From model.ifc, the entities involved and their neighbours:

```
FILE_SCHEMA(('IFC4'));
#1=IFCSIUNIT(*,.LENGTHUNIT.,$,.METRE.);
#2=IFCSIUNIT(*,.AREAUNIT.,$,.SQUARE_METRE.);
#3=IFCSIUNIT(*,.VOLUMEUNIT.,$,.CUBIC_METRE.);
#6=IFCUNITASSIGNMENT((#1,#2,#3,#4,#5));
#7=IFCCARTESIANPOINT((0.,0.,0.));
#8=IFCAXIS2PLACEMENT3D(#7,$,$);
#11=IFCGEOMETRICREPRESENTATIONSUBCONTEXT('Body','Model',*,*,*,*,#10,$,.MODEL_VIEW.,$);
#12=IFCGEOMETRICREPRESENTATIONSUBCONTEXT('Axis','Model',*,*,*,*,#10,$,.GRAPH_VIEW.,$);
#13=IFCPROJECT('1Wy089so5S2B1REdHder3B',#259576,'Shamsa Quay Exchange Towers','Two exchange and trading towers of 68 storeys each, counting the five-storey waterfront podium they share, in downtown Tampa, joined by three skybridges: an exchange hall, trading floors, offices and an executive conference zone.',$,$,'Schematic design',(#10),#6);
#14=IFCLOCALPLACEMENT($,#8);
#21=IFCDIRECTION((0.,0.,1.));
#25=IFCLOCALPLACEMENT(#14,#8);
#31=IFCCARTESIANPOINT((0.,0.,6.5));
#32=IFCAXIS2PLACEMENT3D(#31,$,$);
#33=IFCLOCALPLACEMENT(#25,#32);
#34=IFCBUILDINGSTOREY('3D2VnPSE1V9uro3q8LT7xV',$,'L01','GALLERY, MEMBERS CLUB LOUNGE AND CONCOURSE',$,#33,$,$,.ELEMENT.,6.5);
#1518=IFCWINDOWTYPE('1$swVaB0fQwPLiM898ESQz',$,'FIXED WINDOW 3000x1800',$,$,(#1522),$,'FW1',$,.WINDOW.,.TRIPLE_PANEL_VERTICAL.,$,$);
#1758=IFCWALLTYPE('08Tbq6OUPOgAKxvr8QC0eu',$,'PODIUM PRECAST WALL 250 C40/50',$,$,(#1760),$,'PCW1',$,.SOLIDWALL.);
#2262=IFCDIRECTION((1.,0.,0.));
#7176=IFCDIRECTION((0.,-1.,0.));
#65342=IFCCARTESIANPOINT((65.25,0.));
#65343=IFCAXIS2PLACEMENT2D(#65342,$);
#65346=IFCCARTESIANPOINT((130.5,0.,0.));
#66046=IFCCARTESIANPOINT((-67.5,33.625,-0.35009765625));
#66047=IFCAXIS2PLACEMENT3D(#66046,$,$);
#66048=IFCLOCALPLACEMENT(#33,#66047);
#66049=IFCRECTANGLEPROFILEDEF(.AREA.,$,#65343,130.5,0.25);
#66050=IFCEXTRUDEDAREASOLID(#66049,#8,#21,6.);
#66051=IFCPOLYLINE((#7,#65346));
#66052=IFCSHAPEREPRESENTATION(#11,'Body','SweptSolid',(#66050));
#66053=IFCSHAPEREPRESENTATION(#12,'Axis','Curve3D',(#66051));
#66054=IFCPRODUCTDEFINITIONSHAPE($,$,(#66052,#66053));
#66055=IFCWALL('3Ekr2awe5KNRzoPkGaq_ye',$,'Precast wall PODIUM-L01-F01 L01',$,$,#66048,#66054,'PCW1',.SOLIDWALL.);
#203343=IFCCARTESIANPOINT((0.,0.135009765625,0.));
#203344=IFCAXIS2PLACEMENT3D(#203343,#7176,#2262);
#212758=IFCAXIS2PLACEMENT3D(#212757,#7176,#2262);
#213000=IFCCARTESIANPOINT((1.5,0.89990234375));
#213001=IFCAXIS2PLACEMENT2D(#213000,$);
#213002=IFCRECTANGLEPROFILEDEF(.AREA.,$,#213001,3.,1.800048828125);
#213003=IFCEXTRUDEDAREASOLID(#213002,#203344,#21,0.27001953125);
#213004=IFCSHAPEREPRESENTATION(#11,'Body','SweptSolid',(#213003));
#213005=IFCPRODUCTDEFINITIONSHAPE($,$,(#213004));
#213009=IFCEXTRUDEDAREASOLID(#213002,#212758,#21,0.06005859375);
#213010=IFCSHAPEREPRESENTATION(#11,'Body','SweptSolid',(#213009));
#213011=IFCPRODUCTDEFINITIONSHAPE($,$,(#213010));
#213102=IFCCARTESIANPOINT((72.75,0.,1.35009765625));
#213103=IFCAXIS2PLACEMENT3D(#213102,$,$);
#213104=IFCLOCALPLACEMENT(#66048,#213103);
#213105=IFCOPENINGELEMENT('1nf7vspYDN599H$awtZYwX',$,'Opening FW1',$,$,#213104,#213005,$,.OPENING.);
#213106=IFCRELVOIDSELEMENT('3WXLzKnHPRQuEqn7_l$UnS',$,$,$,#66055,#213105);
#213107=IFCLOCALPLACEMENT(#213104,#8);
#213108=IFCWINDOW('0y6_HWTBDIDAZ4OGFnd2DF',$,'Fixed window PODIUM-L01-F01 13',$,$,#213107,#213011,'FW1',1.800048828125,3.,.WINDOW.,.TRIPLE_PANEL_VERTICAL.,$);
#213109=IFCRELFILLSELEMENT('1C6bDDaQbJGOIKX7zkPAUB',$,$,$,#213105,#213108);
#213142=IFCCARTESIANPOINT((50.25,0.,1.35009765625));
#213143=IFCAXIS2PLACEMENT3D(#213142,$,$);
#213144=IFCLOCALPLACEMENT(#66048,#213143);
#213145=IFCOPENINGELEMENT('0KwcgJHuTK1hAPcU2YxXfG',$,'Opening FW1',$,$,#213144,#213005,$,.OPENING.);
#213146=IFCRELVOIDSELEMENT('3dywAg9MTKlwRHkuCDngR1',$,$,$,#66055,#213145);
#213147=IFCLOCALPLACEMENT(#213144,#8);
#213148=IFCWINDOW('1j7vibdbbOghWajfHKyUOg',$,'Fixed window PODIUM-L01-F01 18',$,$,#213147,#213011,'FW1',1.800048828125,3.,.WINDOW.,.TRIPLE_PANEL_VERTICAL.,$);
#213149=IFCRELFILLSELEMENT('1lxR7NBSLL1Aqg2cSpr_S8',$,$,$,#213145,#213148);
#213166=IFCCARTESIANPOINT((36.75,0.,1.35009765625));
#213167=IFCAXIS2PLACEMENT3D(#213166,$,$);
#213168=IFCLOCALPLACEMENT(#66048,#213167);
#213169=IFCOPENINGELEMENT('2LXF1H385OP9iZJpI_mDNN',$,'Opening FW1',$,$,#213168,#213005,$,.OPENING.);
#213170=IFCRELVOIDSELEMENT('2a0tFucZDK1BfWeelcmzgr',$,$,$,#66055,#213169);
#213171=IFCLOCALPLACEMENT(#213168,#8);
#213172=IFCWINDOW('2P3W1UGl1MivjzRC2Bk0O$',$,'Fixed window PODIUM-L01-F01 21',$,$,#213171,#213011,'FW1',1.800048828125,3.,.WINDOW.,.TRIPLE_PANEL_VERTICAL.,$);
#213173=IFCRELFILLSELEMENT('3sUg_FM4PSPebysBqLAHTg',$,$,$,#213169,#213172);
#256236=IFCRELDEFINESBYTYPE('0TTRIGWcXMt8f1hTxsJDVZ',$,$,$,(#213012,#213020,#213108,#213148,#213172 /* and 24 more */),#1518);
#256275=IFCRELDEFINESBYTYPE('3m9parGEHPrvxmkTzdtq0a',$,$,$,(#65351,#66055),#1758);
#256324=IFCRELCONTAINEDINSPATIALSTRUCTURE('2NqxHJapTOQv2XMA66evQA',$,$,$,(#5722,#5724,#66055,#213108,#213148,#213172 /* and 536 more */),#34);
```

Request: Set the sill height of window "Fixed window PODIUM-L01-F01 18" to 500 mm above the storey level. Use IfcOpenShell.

```python
import numpy as np
import ifcopenshell
import ifcopenshell.api.geometry
import ifcopenshell.geom
import ifcopenshell.util.element
import ifcopenshell.util.placement
import ifcopenshell.util.shape
import ifcopenshell.util.unit

model = ifcopenshell.open("model.ifc")
unit_scale = ifcopenshell.util.unit.calculate_unit_scale(model)

window = model.by_guid("1j7vibdbbOghWajfHKyUOg")
opening = window.FillsVoids[0].RelatingOpeningElement
storey = ifcopenshell.util.element.get_container(window, ifc_class="IfcBuildingStorey")
level = ifcopenshell.util.placement.get_local_placement(storey.ObjectPlacement)[2, 3]

# The opening's origin need not be at the sill, so measure its lowest point.
shape = ifcopenshell.geom.create_shape(ifcopenshell.geom.settings(), opening)
bottom = ifcopenshell.util.shape.get_shape_bottom_elevation(shape, shape.geometry) / unit_scale
dz = level + 0.5 / unit_scale - bottom

shift = np.array([0.0, 0.0, dz])
# The window is placed relative to its opening, so it follows when the opening moves.
matrix = ifcopenshell.util.placement.get_local_placement(opening.ObjectPlacement)
matrix[:3, 3] += shift
ifcopenshell.api.geometry.edit_object_placement(
    model, product=opening, matrix=matrix, is_si=False, should_transform_children=True
)

print(f"moved by {dz * unit_scale:+.3f} m")

model.write("model_v2.ifc")
```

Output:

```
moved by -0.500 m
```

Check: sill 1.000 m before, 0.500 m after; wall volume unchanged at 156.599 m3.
